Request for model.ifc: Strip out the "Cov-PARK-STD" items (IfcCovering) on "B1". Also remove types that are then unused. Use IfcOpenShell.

First a look at what the model holds.

```python
import ifcopenshell
import ifcopenshell.util.element

model = ifcopenshell.open("model.ifc")
print(model.schema)
storey = next(s for s in model.by_type("IfcBuildingStorey") if s.Name == "B1")
coverings = [e for e in ifcopenshell.util.element.get_decomposition(storey) if e.is_a("IfcCovering")]
seen = {}
for e in coverings:
    element_type = ifcopenshell.util.element.get_type(e)
    name = element_type.Name if element_type not in (None, e) else None
    seen[name] = seen.get(name, 0) + 1
for name, count in sorted(seen.items(), key=str):
    print(count, "x", name)
```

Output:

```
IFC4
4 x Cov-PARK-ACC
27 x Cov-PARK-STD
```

```python
import ifcopenshell
import ifcopenshell.api.root
import ifcopenshell.util.element

model = ifcopenshell.open("model.ifc")

storey = next(s for s in model.by_type("IfcBuildingStorey") if s.Name == "B1")
coverings = [e for e in ifcopenshell.util.element.get_decomposition(storey) if e.is_a("IfcCovering")]
targets = [e for e in coverings if (t := ifcopenshell.util.element.get_type(e)) not in (None, e) and t.Name == "Cov-PARK-STD"]
types = {ifcopenshell.util.element.get_type(e) for e in targets} - {None, *targets}

for e in targets:
    ifcopenshell.api.root.remove_product(model, product=e)
print(len(targets), "removed")

unused = [t for t in types if not ifcopenshell.util.element.get_types(t)]
for t in unused:
    ifcopenshell.api.root.remove_product(model, product=t)
print(len(unused), "unused types removed")

model.write("model_edited.ifc")
```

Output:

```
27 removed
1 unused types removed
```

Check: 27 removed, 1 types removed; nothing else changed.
